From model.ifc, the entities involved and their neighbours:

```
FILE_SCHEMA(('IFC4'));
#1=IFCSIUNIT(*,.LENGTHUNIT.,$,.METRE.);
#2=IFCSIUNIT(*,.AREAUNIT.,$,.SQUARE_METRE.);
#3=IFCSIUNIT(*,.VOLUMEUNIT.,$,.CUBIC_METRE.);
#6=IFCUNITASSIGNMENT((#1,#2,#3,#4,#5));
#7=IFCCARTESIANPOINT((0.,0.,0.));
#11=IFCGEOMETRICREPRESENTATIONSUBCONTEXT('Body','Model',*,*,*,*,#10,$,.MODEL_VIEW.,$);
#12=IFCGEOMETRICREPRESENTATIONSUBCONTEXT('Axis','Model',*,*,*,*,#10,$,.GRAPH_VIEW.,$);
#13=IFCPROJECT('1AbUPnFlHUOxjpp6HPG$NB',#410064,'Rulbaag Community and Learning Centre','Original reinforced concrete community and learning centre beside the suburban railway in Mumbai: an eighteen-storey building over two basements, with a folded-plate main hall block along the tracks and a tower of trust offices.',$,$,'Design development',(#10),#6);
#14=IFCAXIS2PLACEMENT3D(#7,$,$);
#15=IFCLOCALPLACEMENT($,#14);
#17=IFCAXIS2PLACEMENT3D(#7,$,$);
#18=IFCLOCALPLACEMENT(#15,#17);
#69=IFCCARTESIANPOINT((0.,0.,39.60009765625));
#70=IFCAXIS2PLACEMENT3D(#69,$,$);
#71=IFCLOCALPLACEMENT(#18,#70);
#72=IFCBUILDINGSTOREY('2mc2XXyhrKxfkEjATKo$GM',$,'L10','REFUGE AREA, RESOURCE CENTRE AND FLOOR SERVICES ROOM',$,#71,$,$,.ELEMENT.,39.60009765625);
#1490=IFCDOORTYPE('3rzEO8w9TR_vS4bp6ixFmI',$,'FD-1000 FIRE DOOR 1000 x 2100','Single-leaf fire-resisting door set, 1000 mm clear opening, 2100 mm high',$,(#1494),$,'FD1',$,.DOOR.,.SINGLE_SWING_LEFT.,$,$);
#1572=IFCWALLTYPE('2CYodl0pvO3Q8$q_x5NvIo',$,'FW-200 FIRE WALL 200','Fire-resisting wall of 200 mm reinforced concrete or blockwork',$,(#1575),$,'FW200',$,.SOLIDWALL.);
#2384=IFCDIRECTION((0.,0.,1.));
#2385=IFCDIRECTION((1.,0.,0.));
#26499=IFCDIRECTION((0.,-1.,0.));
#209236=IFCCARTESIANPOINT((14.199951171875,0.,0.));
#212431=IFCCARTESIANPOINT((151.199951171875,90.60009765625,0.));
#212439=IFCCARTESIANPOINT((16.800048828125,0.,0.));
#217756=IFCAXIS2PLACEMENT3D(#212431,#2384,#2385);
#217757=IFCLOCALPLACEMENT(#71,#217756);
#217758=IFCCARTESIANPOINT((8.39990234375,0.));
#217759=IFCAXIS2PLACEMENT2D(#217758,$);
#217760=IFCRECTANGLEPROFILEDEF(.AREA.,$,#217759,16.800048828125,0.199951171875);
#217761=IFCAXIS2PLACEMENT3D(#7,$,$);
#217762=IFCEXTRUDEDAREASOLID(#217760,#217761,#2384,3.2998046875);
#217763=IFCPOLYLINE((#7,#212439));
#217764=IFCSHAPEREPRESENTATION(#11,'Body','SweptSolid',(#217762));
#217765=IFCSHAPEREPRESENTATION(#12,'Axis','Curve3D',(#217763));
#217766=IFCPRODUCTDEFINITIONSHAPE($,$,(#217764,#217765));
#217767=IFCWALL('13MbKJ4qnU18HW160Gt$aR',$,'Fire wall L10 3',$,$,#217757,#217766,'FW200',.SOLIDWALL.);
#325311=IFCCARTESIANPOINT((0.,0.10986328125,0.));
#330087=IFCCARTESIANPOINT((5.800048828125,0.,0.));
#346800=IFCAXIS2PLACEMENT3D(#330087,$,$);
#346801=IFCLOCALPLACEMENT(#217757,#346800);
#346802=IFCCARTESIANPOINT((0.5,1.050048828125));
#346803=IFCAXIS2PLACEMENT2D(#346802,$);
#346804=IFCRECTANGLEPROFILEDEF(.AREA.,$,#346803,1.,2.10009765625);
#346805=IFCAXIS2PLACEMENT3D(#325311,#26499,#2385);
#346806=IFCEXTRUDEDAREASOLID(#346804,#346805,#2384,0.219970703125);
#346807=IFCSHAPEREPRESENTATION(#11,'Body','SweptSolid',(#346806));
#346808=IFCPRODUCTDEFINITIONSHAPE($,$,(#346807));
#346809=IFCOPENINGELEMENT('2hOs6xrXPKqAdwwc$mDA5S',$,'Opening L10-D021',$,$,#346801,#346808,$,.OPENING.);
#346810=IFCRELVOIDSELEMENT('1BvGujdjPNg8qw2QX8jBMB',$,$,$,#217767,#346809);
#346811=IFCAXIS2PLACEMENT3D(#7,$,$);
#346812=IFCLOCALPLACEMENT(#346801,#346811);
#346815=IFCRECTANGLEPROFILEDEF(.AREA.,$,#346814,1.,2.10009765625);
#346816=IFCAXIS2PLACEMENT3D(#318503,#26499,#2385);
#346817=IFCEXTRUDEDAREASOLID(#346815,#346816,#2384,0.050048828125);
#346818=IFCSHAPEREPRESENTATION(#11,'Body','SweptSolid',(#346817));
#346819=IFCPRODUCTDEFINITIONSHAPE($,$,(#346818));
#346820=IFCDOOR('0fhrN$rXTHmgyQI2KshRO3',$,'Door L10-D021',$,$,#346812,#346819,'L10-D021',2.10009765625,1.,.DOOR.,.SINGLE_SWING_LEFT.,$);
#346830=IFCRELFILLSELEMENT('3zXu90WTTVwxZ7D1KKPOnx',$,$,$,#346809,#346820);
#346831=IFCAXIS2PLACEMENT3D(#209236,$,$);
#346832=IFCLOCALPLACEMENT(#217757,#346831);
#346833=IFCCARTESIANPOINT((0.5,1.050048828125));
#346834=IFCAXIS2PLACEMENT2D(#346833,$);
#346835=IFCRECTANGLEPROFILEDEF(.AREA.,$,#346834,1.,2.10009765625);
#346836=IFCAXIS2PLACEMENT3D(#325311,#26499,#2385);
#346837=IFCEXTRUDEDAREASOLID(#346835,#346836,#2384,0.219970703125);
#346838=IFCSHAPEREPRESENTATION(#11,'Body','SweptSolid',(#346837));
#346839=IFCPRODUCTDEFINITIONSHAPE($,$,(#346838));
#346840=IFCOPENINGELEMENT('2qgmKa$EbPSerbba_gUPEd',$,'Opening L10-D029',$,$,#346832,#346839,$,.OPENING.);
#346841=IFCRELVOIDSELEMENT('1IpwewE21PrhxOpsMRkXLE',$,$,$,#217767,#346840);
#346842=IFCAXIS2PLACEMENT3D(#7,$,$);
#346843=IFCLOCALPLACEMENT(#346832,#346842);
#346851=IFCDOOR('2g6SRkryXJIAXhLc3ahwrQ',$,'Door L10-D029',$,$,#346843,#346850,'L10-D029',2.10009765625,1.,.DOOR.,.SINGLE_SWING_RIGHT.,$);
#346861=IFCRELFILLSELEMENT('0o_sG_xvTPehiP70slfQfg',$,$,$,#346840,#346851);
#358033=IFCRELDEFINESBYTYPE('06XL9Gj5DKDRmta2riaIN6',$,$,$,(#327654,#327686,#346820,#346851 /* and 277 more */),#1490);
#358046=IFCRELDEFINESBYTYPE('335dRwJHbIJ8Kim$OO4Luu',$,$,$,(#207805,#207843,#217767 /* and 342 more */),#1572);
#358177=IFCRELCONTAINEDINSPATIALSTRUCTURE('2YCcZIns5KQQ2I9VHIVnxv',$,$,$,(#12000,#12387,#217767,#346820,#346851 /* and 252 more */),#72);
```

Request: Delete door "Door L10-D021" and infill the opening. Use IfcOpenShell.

```python
import ifcopenshell
import ifcopenshell.api.feature
import ifcopenshell.api.root
import ifcopenshell.geom
import ifcopenshell.util.shape

model = ifcopenshell.open("model.ifc")
settings = ifcopenshell.geom.settings()


def volume(element):
    """Net volume in cubic metres, openings subtracted."""
    shape = ifcopenshell.geom.create_shape(settings, element)
    return ifcopenshell.util.shape.get_volume(shape.geometry)


door = model.by_guid("0fhrN$rXTHmgyQI2KshRO3")
opening = door.FillsVoids[0].RelatingOpeningElement
wall = opening.VoidsElements[0].RelatingBuildingElement
before = volume(wall)

ifcopenshell.api.root.remove_product(model, product=door)
ifcopenshell.api.feature.remove_feature(model, feature=opening)

after = volume(wall)

print(f"wall volume {before:.3f} -> {after:.3f} m3")

model.write("model_rev.ifc")
```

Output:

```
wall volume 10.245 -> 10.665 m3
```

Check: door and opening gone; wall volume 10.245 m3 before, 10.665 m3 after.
